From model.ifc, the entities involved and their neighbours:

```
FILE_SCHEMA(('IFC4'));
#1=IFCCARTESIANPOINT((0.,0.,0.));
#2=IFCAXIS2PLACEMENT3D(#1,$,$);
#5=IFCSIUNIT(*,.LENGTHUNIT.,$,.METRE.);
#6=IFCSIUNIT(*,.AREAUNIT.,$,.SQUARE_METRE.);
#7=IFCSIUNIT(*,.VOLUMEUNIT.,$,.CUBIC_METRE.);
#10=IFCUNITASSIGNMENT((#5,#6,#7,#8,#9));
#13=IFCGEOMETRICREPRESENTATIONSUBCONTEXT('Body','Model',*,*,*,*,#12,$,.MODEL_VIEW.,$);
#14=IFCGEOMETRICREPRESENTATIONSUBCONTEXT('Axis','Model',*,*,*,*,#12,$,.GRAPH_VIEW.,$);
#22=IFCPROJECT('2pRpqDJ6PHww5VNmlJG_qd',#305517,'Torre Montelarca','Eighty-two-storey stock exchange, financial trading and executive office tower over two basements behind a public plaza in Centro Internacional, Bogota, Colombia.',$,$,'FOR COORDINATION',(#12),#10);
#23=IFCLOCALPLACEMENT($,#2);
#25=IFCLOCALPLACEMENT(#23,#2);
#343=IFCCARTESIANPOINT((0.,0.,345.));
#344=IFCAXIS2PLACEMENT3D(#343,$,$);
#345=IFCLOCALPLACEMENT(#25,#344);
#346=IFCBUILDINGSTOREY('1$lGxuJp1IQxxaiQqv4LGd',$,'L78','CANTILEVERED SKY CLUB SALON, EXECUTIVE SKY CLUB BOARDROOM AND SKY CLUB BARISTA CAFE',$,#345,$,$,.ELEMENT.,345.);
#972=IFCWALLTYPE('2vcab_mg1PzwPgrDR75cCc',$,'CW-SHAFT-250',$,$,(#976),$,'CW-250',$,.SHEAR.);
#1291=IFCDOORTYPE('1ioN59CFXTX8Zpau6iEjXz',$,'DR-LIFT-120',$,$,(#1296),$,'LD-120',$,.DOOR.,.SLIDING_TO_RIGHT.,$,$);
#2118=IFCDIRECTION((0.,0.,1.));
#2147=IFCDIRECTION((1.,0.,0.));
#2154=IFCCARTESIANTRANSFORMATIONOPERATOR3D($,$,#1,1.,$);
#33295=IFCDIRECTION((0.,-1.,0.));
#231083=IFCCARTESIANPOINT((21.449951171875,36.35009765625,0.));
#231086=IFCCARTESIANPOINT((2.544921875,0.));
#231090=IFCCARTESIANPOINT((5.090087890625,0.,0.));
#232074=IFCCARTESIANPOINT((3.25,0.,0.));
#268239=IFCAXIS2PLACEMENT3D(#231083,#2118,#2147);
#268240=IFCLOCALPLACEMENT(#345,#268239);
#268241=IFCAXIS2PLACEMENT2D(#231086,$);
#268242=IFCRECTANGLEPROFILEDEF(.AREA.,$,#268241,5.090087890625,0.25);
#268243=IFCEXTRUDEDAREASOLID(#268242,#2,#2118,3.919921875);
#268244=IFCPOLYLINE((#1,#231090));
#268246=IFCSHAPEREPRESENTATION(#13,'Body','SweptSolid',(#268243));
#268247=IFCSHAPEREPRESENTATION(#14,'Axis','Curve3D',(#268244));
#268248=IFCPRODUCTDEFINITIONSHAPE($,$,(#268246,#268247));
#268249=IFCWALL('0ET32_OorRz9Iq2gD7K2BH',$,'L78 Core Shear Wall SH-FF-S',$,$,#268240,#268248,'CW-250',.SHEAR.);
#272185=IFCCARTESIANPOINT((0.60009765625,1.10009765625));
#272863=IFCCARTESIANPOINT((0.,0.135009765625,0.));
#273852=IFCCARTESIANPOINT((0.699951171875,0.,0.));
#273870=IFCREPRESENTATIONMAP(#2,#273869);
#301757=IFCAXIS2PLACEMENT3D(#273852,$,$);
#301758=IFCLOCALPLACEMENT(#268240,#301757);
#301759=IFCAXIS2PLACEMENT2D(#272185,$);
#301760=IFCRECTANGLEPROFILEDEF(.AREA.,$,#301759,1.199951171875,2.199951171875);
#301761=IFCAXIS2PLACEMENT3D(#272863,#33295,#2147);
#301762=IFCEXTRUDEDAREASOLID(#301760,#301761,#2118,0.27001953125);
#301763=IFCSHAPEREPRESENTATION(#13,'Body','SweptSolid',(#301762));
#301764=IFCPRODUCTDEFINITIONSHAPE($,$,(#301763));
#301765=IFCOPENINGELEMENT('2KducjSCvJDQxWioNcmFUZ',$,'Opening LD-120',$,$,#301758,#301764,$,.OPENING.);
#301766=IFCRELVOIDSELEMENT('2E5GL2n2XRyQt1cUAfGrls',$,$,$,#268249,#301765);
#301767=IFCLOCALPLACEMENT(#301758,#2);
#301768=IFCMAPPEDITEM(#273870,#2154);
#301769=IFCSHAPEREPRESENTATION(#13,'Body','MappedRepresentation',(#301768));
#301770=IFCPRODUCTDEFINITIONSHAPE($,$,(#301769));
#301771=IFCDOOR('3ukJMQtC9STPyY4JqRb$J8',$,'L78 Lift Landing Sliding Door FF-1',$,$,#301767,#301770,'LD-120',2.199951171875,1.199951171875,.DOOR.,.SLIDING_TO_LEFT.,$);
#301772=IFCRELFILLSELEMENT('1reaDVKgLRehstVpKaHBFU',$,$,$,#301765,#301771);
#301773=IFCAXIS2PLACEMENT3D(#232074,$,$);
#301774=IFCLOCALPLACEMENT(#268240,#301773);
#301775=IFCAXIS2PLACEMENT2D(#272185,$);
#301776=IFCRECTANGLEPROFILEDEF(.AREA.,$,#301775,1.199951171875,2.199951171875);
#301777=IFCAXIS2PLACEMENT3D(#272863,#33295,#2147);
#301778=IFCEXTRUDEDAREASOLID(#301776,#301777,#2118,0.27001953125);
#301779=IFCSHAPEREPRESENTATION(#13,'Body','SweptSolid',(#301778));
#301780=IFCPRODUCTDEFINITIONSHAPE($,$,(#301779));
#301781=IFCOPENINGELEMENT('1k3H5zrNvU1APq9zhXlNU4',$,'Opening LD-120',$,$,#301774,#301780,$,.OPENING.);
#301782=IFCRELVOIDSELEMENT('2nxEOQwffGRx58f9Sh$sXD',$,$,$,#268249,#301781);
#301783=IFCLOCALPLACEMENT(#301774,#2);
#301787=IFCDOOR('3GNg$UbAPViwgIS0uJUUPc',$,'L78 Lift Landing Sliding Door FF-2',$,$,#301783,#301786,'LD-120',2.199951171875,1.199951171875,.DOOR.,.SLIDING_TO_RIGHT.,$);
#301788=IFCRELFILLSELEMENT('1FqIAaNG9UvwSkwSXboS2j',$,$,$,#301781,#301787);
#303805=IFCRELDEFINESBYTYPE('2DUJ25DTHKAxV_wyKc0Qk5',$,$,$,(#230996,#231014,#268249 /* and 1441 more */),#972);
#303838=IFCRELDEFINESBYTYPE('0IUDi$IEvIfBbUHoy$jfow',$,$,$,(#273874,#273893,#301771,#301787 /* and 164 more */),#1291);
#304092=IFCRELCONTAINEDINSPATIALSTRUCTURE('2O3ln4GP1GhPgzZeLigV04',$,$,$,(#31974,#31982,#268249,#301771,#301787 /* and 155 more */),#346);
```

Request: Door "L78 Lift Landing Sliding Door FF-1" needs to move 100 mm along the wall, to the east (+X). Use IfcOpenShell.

```python
import ifcopenshell
import ifcopenshell.api.geometry
import ifcopenshell.util.placement
import ifcopenshell.util.unit

model = ifcopenshell.open("model.ifc")
unit_scale = ifcopenshell.util.unit.calculate_unit_scale(model)

door = model.by_guid("3ukJMQtC9STPyY4JqRb$J8")
opening = door.FillsVoids[0].RelatingOpeningElement
wall = opening.VoidsElements[0].RelatingBuildingElement

wall_matrix = ifcopenshell.util.placement.get_local_placement(wall.ObjectPlacement)
shift = wall_matrix[:3, 0] * 0.1 / unit_scale
before = ifcopenshell.util.placement.get_local_placement(door.ObjectPlacement)[:3, 3].copy()

# The door is placed relative to its opening, so it follows when the opening moves.
matrix = ifcopenshell.util.placement.get_local_placement(opening.ObjectPlacement)
matrix[:3, 3] += shift
ifcopenshell.api.geometry.edit_object_placement(
    model, product=opening, matrix=matrix, is_si=False, should_transform_children=True
)

after = ifcopenshell.util.placement.get_local_placement(door.ObjectPlacement)[:3, 3]
print("door moved by", (after - before).round(3) + 0.0)

model.write("model_rev.ifc")
```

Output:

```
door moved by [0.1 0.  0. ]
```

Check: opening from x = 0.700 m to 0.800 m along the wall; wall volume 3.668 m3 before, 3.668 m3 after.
